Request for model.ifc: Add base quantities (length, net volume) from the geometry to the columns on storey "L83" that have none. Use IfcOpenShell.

First a look at what the model holds.

```python
import ifcopenshell
import ifcopenshell.util.element
import ifcopenshell.util.unit

model = ifcopenshell.open("model.ifc")
print(model.schema)
for unit_type in ("LENGTHUNIT", "AREAUNIT", "VOLUMEUNIT"):
    print(unit_type, ifcopenshell.util.unit.calculate_unit_scale(model, unit_type))
storey = next(s for s in model.by_type("IfcBuildingStorey") if s.Name == "L83")
columns = [e for e in ifcopenshell.util.element.get_decomposition(storey) if e.is_a("IfcColumn")]
for e in sorted(columns, key=lambda e: e.id()):
    print(e.id(), e.is_a(), e.Name, list(ifcopenshell.util.element.get_psets(e, qtos_only=True)), sep=" | ")
```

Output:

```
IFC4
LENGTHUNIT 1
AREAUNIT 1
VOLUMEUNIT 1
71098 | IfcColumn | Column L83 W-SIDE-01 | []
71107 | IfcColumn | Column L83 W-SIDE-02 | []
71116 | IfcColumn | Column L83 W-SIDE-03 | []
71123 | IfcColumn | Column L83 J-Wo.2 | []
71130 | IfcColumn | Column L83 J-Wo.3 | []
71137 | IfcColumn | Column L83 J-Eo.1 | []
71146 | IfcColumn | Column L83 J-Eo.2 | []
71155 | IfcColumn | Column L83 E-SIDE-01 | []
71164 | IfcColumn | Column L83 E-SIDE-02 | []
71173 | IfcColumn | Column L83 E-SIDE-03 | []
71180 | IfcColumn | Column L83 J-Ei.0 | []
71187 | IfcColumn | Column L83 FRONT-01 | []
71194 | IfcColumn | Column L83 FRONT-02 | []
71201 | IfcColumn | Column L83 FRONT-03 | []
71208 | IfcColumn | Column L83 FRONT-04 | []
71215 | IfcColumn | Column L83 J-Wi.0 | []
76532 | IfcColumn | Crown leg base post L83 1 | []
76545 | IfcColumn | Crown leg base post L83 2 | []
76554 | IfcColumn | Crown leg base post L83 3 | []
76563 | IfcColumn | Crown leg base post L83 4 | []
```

```python
import ifcopenshell
import ifcopenshell.api.pset
import ifcopenshell.geom
import ifcopenshell.util.element
import ifcopenshell.util.shape
import ifcopenshell.util.unit

model = ifcopenshell.open("model.ifc")
unit_scale = ifcopenshell.util.unit.calculate_unit_scale(model)
volume_scale = ifcopenshell.util.unit.calculate_unit_scale(model, "VOLUMEUNIT")
settings = ifcopenshell.geom.settings()

storey = next(s for s in model.by_type("IfcBuildingStorey") if s.Name == "L83")
columns = [e for e in ifcopenshell.util.element.get_decomposition(storey) if e.is_a("IfcColumn")]

for e in sorted(columns, key=lambda e: e.id()):
    if ifcopenshell.util.element.get_psets(e, qtos_only=True, should_inherit=False):
        continue
    # Geometry comes back in metres, in the element's own axes.
    shape = ifcopenshell.geom.create_shape(settings, e)
    values = {
        "Length": ifcopenshell.util.shape.get_z(shape.geometry) / unit_scale,
        "NetVolume": ifcopenshell.util.shape.get_volume(shape.geometry) / volume_scale,
    }
    qto = ifcopenshell.api.pset.add_qto(model, product=e, name="Qto_ColumnBaseQuantities")
    ifcopenshell.api.pset.edit_qto(model, qto=qto, properties=values)
    print(e.id(), {k: round(v, 3) for k, v in values.items()})

model.write("model_edited.ifc")
```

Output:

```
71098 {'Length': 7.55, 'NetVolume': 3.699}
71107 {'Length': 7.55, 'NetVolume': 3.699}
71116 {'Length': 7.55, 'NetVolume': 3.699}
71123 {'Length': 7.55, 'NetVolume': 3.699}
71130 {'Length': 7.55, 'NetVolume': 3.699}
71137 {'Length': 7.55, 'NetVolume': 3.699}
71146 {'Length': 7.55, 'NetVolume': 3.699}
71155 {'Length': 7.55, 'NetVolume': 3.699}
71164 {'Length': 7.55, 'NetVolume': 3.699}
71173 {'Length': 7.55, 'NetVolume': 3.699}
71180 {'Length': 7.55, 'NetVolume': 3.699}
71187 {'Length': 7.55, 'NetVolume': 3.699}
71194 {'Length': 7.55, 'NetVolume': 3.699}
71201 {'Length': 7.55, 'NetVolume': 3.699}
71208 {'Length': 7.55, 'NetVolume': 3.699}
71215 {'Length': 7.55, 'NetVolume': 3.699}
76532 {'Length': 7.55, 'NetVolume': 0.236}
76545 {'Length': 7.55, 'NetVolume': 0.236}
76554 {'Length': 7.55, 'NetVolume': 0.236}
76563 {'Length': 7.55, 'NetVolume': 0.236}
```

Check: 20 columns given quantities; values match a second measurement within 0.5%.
